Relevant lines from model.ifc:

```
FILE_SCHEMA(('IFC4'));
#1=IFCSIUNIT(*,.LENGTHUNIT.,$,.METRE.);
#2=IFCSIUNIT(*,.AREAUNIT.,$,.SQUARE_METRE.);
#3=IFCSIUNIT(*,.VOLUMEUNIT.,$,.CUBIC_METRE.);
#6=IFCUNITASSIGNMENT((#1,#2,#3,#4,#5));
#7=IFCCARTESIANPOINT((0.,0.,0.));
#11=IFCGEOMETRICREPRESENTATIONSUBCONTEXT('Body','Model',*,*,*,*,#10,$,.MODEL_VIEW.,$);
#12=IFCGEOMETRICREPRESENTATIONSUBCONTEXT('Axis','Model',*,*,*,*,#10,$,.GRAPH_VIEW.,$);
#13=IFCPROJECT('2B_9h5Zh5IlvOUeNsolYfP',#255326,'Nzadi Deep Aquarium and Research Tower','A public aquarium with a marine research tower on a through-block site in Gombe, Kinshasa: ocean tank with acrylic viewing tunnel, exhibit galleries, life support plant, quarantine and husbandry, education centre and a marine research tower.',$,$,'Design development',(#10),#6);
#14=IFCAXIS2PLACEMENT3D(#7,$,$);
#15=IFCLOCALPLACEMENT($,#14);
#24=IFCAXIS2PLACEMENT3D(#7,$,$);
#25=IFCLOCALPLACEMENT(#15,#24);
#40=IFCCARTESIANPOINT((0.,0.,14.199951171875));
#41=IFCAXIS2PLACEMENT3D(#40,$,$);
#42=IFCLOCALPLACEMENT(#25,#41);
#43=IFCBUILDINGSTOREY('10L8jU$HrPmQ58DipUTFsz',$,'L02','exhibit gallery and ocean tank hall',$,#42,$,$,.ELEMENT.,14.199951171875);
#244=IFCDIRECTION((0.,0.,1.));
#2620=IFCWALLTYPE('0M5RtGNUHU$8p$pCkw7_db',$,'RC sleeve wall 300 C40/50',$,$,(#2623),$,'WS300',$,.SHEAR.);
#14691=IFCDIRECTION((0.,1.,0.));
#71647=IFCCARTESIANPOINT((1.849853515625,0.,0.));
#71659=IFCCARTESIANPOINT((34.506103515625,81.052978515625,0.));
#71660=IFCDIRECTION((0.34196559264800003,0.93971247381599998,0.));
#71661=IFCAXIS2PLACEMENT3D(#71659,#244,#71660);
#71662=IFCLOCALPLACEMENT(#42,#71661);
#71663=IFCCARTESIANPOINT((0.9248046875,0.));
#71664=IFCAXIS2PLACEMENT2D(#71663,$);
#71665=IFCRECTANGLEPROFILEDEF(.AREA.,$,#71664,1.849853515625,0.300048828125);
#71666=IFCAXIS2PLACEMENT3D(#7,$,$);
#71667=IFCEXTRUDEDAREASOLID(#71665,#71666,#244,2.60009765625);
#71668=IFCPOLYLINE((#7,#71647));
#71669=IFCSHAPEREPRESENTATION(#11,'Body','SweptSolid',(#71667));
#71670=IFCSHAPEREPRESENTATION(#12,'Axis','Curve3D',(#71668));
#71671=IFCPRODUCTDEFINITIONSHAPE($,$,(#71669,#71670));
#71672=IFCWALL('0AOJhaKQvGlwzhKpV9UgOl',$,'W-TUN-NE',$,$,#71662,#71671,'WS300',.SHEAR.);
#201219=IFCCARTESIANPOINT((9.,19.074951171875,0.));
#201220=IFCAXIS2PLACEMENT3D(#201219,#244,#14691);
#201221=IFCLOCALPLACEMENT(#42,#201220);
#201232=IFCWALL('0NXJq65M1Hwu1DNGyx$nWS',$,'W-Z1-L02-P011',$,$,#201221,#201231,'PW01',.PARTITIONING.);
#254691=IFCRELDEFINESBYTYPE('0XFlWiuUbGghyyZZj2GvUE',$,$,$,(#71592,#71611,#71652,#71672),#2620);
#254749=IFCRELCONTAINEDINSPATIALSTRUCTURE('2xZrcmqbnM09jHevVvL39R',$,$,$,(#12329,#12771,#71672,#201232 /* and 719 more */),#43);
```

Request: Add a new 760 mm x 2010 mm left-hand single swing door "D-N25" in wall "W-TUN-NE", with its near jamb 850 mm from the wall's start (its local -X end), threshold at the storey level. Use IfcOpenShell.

```python
import numpy as np
import ifcopenshell
import ifcopenshell.api.feature
import ifcopenshell.api.geometry
import ifcopenshell.api.root
import ifcopenshell.api.spatial
import ifcopenshell.geom
import ifcopenshell.util.element
import ifcopenshell.util.placement
import ifcopenshell.util.representation
import ifcopenshell.util.shape
import ifcopenshell.util.unit

model = ifcopenshell.open("model.ifc")
unit_scale = ifcopenshell.util.unit.calculate_unit_scale(model)
settings = ifcopenshell.geom.settings()


def volume(element):
    """Net volume in cubic metres, openings subtracted."""
    shape = ifcopenshell.geom.create_shape(settings, element)
    return ifcopenshell.util.shape.get_volume(shape.geometry)


wall = model.by_guid("0AOJhaKQvGlwzhKpV9UgOl")
storey = ifcopenshell.util.element.get_container(wall, ifc_class="IfcBuildingStorey")
context = ifcopenshell.util.representation.get_context(model, "Model", "Body", "MODEL_VIEW")
before = volume(wall)

width, height, from_end, sill = 0.76, 2.01, 0.85, 0.0  # metres

# The wall runs along its own X axis, and the end named is its -X end.
wall_shape = ifcopenshell.geom.create_shape(settings, wall)
x, y, z = ifcopenshell.util.shape.get_vertices(wall_shape.geometry).T
start = x.min() + from_end
face, thickness = float(y.min()), float(y.max() - y.min())
wall_matrix = ifcopenshell.util.placement.get_local_placement(wall.ObjectPlacement)
level = ifcopenshell.util.placement.get_local_placement(storey.ObjectPlacement)[2, 3]


def in_wall(x, y):
    """Placement at x, y metres in the wall's axes, at sill height."""
    matrix = wall_matrix.copy()
    matrix[:, 3] = wall_matrix @ np.array([x / unit_scale, y / unit_scale, 0.0, 1.0])
    matrix[2, 3] = level + sill / unit_scale
    return matrix


# Opening: a box that overshoots both wall faces by 50 mm.
opening = ifcopenshell.api.root.create_entity(model, ifc_class="IfcOpeningElement", predefined_type="OPENING")
box = ifcopenshell.api.geometry.add_wall_representation(
    model, context=context, length=width, height=height, thickness=thickness + 0.1
)
ifcopenshell.api.geometry.assign_representation(model, product=opening, representation=box)
ifcopenshell.api.geometry.edit_object_placement(model, product=opening, matrix=in_wall(start, face - 0.05), is_si=False)
ifcopenshell.api.feature.add_feature(model, feature=opening, element=wall)

door = ifcopenshell.api.root.create_entity(model, ifc_class="IfcDoor", name="D-N25", predefined_type="DOOR")
door.OverallWidth, door.OverallHeight = width / unit_scale, height / unit_scale
door.OperationType = "SINGLE_SWING_LEFT"
body = ifcopenshell.api.geometry.add_door_representation(
    model,
    context=context,
    overall_width=door.OverallWidth,
    overall_height=door.OverallHeight,
    operation_type="SINGLE_SWING_LEFT",
    lining_properties={"LiningDepth": thickness / unit_scale, "ThresholdDepth": thickness / unit_scale},
)
ifcopenshell.api.geometry.assign_representation(model, product=door, representation=body)
ifcopenshell.api.spatial.assign_container(model, products=[door], relating_structure=storey)
ifcopenshell.api.feature.add_filling(model, opening=opening, element=door)

# The lining spans the wall, so the door starts at the wall face.
ifcopenshell.api.geometry.edit_object_placement(model, product=door, matrix=in_wall(start, face), is_si=False)

after = volume(wall)

print(f"wall volume {before:.3f} -> {after:.3f} m3")

model.write("model-out.ifc")
```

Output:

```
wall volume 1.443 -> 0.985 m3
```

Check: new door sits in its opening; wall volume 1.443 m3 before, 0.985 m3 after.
